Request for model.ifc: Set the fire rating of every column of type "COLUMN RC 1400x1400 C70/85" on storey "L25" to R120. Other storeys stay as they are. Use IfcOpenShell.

First a look at what the model holds.

```python
import ifcopenshell
import ifcopenshell.util.element

model = ifcopenshell.open("model.ifc")
print(model.schema)
storey = next(s for s in model.by_type("IfcBuildingStorey") if s.Name == "L25")
columns = [e for e in ifcopenshell.util.element.get_decomposition(storey) if e.is_a("IfcColumn")]
seen = {}
for e in columns:
    element_type = ifcopenshell.util.element.get_type(e)
    key = (element_type.Name if element_type != e and element_type else None, ifcopenshell.util.element.get_pset(e, "Pset_ColumnCommon", "FireRating"))
    seen[key] = seen.get(key, 0) + 1
for (name, value), count in sorted(seen.items(), key=str):
    print(count, "x", name, "|", value)
```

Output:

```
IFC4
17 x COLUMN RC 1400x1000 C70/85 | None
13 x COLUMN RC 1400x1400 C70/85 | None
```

```python
import ifcopenshell
import ifcopenshell.api.pset
import ifcopenshell.util.element

model = ifcopenshell.open("model.ifc")

storey = next(s for s in model.by_type("IfcBuildingStorey") if s.Name == "L25")
columns = [e for e in ifcopenshell.util.element.get_decomposition(storey) if e.is_a("IfcColumn")]

count = 0
for e in columns:
    element_type = ifcopenshell.util.element.get_type(e)
    if element_type in (None, e) or element_type.Name != "COLUMN RC 1400x1400 C70/85":
        continue
    found = ifcopenshell.util.element.get_pset(e, "Pset_ColumnCommon", should_inherit=False)
    if found:
        pset = model.by_id(found["id"])
        if len(ifcopenshell.util.element.get_elements_by_pset(pset)) > 1:
            pset = ifcopenshell.api.pset.unshare_pset(model, products=[e], pset=pset)[0]
    else:
        pset = ifcopenshell.api.pset.add_pset(model, product=e, name="Pset_ColumnCommon")
    ifcopenshell.api.pset.edit_pset(model, pset=pset, properties={"FireRating": "R120"})
    count += 1

print(count, "columns updated")

model.write("model-out.ifc")
```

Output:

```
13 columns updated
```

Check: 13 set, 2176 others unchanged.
